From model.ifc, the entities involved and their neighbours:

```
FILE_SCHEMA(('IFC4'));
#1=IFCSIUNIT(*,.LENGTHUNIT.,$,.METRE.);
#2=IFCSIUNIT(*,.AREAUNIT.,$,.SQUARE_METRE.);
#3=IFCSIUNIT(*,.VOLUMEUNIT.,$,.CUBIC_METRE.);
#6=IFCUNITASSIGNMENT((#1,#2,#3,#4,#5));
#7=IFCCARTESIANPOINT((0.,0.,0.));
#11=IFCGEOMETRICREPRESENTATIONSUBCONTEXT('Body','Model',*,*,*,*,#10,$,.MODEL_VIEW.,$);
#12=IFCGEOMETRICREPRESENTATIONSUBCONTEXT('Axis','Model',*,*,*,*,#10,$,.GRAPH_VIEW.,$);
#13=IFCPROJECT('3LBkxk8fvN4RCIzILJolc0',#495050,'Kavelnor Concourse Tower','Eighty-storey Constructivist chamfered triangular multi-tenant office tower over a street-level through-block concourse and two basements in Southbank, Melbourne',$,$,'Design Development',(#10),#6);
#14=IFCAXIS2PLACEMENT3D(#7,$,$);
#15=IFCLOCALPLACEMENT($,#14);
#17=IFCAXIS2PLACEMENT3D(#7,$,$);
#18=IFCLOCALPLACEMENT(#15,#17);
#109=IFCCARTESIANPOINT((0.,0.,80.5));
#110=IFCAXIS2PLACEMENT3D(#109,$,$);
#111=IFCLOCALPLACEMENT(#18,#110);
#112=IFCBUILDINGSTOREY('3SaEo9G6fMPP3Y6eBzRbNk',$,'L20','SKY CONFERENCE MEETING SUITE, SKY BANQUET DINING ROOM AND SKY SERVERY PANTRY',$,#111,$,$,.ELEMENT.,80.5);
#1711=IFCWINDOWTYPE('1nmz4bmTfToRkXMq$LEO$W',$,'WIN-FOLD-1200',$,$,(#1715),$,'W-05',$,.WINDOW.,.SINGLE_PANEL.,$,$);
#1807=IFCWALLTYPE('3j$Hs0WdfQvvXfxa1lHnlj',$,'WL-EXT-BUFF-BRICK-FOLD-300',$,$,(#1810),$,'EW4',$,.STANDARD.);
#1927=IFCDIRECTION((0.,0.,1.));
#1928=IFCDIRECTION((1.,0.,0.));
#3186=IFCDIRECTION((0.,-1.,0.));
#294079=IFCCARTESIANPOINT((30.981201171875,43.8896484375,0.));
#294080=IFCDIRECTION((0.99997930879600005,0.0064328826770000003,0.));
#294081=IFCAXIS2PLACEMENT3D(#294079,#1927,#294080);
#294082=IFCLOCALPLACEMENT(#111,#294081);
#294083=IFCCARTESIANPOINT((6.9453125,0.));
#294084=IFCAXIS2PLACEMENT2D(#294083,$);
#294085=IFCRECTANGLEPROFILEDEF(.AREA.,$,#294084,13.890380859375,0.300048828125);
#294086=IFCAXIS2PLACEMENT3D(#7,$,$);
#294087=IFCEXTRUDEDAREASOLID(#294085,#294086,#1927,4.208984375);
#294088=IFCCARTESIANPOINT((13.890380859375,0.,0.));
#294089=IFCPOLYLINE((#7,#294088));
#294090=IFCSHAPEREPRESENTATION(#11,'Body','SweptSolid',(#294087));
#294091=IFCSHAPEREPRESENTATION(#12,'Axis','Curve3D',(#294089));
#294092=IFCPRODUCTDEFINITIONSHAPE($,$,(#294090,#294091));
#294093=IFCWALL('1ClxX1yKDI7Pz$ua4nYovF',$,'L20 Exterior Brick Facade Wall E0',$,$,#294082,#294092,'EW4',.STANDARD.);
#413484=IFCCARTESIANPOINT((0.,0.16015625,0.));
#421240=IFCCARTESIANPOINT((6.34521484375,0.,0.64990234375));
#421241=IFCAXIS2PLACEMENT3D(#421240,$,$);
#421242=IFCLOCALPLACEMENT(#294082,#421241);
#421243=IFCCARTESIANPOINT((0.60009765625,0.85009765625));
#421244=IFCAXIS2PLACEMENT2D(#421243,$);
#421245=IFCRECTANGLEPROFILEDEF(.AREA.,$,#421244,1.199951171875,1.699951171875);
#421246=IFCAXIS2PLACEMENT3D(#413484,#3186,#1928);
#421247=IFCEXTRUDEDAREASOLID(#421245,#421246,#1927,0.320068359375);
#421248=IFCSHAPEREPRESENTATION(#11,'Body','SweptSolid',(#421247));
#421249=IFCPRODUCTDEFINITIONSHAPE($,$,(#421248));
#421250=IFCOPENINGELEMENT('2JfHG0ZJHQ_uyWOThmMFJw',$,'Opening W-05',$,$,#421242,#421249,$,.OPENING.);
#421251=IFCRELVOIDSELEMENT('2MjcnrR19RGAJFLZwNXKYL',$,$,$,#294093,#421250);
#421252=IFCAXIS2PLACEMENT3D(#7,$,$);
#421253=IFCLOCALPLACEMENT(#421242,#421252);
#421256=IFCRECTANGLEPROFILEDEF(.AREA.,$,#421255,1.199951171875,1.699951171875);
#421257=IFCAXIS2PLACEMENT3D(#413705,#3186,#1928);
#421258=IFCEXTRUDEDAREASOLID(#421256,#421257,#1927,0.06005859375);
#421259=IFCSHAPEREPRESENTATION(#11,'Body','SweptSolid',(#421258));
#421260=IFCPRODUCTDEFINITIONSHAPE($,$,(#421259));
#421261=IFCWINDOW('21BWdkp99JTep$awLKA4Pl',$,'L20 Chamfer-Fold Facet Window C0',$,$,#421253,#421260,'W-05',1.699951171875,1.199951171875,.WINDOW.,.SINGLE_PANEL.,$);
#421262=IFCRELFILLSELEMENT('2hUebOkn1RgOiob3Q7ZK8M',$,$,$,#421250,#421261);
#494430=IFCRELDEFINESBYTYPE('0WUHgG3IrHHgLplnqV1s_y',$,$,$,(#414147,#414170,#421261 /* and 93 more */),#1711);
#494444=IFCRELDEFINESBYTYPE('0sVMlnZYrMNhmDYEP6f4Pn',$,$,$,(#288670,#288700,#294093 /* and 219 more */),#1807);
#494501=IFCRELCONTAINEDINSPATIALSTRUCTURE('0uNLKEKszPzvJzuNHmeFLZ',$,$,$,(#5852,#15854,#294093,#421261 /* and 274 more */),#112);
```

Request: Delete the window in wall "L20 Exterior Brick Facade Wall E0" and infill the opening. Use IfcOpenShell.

```python
import ifcopenshell
import ifcopenshell.api.feature
import ifcopenshell.api.root
import ifcopenshell.geom
import ifcopenshell.util.shape

model = ifcopenshell.open("model.ifc")
settings = ifcopenshell.geom.settings()


def volume(element):
    """Net volume in cubic metres, openings subtracted."""
    shape = ifcopenshell.geom.create_shape(settings, element)
    return ifcopenshell.util.shape.get_volume(shape.geometry)


window = model.by_guid("21BWdkp99JTep$awLKA4Pl")
opening = window.FillsVoids[0].RelatingOpeningElement
wall = opening.VoidsElements[0].RelatingBuildingElement
before = volume(wall)

ifcopenshell.api.root.remove_product(model, product=window)
ifcopenshell.api.feature.remove_feature(model, feature=opening)

after = volume(wall)

print(f"wall volume {before:.3f} -> {after:.3f} m3")

model.write("model_edited.ifc")
```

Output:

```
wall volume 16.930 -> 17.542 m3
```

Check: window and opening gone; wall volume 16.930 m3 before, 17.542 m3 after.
